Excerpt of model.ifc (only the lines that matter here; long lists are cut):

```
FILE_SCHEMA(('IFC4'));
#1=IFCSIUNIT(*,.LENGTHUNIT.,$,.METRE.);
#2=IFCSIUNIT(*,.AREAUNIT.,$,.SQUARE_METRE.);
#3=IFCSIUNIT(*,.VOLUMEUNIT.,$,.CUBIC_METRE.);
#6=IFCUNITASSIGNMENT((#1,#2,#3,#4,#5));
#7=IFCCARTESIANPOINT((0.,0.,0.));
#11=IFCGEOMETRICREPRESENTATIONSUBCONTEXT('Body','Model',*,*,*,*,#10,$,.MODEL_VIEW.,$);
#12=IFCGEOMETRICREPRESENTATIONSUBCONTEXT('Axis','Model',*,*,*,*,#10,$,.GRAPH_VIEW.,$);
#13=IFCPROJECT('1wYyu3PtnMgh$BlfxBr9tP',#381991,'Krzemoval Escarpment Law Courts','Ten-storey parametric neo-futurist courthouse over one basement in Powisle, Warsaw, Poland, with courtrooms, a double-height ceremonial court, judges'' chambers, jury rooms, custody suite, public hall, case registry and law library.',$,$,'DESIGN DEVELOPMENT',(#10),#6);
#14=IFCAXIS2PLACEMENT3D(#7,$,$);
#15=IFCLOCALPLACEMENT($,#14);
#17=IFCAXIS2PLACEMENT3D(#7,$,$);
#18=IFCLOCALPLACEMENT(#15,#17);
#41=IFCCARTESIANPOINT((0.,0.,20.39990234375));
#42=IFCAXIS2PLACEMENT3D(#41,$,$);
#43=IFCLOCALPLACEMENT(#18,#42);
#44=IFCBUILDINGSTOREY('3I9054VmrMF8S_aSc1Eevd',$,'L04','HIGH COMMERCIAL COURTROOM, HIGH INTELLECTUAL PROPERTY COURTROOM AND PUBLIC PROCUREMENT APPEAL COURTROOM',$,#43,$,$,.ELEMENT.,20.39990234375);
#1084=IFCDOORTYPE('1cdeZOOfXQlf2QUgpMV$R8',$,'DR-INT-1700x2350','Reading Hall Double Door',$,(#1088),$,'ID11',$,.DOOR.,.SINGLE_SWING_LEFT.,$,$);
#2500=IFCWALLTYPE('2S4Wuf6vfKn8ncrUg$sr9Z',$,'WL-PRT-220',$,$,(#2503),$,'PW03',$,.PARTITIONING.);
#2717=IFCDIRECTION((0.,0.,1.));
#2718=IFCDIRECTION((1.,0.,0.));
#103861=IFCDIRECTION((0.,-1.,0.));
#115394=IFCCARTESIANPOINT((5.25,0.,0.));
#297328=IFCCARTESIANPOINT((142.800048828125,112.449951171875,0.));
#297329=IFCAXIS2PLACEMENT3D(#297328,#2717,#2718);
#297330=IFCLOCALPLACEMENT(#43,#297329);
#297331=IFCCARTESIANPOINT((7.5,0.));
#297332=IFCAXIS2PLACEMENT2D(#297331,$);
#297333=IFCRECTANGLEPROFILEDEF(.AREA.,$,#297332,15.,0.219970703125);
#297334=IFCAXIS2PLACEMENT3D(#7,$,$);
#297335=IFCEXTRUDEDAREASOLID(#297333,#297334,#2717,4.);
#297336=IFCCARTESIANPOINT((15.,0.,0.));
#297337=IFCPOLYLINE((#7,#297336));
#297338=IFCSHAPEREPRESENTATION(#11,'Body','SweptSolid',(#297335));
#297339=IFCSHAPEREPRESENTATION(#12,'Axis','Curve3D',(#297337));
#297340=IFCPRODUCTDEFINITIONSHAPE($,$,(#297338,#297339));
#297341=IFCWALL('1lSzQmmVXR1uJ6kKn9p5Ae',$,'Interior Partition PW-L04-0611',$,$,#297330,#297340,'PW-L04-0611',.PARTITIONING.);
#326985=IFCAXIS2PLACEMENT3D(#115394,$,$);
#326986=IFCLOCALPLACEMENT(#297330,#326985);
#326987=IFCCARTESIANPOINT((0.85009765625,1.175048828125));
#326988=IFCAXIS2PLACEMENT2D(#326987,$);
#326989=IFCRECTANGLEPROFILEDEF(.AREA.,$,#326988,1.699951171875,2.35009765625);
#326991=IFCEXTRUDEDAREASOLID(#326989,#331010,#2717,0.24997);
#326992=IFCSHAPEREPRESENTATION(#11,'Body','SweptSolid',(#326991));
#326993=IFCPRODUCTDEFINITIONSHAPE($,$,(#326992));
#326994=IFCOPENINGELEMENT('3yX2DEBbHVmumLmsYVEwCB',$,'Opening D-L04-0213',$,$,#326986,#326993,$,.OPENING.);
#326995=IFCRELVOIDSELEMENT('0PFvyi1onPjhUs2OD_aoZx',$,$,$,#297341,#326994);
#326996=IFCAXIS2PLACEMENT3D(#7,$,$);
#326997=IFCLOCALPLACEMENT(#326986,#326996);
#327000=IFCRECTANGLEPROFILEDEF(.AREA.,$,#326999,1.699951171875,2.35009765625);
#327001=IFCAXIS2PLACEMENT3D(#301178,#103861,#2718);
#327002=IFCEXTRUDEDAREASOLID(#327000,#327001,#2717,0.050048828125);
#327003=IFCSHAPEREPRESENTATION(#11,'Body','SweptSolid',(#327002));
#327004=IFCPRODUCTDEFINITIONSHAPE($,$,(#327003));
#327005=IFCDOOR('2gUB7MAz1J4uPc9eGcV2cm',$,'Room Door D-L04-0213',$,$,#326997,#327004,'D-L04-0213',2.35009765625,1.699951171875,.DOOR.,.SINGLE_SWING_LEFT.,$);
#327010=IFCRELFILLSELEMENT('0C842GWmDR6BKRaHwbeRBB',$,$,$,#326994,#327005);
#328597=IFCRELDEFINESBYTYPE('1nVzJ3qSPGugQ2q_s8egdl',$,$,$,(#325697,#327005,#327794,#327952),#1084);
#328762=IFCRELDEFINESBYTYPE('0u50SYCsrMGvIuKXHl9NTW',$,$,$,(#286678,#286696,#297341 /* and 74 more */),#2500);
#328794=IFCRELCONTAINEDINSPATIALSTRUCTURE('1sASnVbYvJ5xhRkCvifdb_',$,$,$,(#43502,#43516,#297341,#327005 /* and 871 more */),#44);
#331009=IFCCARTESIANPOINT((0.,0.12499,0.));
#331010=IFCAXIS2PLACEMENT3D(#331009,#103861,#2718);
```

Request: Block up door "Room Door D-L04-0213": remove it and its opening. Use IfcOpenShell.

```python
import ifcopenshell
import ifcopenshell.api.feature
import ifcopenshell.api.root
import ifcopenshell.geom
import ifcopenshell.util.shape

model = ifcopenshell.open("model.ifc")
settings = ifcopenshell.geom.settings()


def volume(element):
    """Net volume in cubic metres, openings subtracted."""
    shape = ifcopenshell.geom.create_shape(settings, element)
    return ifcopenshell.util.shape.get_volume(shape.geometry)


door = model.by_id(327005)
opening = door.FillsVoids[0].RelatingOpeningElement
wall = opening.VoidsElements[0].RelatingBuildingElement
before = volume(wall)

ifcopenshell.api.root.remove_product(model, product=door)
ifcopenshell.api.feature.remove_feature(model, feature=opening)

after = volume(wall)

print(f"wall volume {before:.3f} -> {after:.3f} m3")

model.write("model-out.ifc")
```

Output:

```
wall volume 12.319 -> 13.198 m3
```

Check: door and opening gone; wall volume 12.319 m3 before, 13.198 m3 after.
